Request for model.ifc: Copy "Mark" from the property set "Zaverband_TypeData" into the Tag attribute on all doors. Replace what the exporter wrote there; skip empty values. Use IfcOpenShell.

First a look at what the model holds.

```python
import ifcopenshell
import ifcopenshell.util.element

model = ifcopenshell.open("model.ifc")
print(model.schema)
doors = model.by_type("IfcDoor")
print(len(doors), "doors")
for e in doors[:8]:
    source = ifcopenshell.util.element.get_pset(e, "Zaverband_TypeData", "Mark")
    target = e.Tag
    print(e.id(), repr(source), repr(target), sep=" | ")
```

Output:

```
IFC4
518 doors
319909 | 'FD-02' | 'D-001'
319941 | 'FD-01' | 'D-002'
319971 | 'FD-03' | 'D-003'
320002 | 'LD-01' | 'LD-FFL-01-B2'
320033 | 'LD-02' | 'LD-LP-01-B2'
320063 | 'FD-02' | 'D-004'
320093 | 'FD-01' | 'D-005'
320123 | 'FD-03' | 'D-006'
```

```python
import ifcopenshell
import ifcopenshell.util.element

model = ifcopenshell.open("model.ifc")

count = 0
for e in model.by_type("IfcDoor"):
    value = ifcopenshell.util.element.get_pset(e, "Zaverband_TypeData", "Mark")
    current = e.Tag
    if not value or not value.strip() or current == value:
        continue
    e.Tag = value
    count += 1

print(count, "doors updated")

model.write("model_rev.ifc")
```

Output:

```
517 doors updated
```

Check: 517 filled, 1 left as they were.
